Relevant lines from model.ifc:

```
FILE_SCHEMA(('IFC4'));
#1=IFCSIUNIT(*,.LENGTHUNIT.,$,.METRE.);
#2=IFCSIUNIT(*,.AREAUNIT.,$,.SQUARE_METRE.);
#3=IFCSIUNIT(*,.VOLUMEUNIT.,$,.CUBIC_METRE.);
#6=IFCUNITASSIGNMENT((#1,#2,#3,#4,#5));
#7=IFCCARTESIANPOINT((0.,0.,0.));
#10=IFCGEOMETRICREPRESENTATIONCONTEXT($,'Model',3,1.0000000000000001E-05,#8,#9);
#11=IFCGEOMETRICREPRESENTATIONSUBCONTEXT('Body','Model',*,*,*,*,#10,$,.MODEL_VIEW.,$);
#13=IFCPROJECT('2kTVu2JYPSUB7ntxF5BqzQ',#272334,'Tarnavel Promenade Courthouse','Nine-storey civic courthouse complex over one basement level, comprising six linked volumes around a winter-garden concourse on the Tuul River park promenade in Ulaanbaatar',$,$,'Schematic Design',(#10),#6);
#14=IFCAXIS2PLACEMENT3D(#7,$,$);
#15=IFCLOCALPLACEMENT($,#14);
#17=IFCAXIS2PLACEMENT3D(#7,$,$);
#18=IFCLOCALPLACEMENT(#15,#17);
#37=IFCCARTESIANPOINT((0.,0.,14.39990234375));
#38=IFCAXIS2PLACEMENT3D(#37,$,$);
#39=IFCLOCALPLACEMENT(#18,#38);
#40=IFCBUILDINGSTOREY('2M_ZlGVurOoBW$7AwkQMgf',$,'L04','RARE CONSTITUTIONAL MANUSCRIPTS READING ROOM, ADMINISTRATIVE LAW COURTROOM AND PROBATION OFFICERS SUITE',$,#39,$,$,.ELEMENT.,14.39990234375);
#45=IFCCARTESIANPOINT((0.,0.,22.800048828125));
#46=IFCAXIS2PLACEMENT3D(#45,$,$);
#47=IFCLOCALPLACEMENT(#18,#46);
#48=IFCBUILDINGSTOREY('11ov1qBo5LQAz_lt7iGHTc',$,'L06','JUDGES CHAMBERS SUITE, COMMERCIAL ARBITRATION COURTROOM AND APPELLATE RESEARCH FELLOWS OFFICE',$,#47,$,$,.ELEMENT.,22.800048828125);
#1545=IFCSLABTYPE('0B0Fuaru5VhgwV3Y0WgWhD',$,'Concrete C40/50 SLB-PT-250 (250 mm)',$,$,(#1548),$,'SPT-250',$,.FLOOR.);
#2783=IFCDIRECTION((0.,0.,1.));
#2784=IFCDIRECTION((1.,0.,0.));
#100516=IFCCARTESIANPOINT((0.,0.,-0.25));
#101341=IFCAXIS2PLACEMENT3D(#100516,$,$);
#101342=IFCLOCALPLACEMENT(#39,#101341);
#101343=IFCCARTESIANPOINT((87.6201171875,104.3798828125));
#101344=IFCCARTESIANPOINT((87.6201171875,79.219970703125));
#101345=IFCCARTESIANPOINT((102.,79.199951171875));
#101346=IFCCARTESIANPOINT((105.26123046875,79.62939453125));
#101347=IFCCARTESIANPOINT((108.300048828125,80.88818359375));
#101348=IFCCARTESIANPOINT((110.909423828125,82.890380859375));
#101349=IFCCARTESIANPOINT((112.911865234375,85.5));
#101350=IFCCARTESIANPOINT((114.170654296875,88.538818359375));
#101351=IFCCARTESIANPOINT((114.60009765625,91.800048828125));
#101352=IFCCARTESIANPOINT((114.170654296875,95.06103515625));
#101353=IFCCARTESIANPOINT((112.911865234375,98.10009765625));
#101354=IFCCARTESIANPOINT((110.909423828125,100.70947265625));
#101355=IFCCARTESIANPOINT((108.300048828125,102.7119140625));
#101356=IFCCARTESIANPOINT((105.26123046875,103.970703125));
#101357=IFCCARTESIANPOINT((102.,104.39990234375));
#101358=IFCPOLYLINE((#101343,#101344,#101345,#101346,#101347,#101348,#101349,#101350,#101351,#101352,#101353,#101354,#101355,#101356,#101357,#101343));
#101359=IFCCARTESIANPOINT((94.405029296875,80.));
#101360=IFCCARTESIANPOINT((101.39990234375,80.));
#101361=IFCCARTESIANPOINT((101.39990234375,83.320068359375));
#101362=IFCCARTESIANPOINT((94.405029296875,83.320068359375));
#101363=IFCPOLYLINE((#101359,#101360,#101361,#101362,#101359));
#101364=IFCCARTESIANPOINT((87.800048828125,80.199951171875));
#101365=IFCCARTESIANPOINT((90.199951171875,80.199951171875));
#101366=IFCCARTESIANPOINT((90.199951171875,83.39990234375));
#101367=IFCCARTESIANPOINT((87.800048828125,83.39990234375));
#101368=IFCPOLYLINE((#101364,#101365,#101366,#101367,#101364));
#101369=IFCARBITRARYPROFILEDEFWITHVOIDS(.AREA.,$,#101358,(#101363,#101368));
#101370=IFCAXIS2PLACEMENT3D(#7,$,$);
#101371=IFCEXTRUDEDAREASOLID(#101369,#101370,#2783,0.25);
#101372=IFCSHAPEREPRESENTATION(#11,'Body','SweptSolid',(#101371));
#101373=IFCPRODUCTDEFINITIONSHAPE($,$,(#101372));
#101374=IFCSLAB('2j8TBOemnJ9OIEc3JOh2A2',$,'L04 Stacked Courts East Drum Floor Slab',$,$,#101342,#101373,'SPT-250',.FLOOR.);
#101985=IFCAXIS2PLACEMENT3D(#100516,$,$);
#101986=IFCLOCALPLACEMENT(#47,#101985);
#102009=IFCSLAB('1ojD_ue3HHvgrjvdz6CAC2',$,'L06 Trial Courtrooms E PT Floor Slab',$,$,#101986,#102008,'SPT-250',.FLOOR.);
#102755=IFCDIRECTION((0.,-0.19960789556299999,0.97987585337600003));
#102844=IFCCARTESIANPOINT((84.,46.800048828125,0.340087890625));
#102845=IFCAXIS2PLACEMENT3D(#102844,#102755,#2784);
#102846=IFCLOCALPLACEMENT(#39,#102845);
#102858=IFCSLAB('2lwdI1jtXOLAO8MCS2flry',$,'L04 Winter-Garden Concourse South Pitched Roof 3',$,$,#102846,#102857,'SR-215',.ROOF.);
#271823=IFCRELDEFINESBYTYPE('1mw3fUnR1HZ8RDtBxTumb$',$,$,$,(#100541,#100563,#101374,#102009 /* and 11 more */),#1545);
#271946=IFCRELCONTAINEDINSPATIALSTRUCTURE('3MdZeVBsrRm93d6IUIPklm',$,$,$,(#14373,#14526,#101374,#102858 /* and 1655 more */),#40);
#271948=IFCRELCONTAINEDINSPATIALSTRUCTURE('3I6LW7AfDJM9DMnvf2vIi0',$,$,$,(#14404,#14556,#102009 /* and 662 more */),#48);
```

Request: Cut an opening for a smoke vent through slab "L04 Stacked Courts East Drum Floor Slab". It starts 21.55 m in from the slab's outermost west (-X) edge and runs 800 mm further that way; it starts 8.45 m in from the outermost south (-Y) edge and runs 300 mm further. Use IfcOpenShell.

```python
import numpy as np
import ifcopenshell
import ifcopenshell.api.feature
import ifcopenshell.api.geometry
import ifcopenshell.api.root
import ifcopenshell.geom
import ifcopenshell.util.placement
import ifcopenshell.util.representation
import ifcopenshell.util.shape
import ifcopenshell.util.unit

model = ifcopenshell.open("model.ifc")
unit_scale = ifcopenshell.util.unit.calculate_unit_scale(model)
settings = ifcopenshell.geom.settings()


def volume(element):
    """Net volume in cubic metres, openings subtracted."""
    shape = ifcopenshell.geom.create_shape(settings, element)
    return ifcopenshell.util.shape.get_volume(shape.geometry)


slab = model.by_guid("2j8TBOemnJ9OIEc3JOh2A2")
before = volume(slab)

# Extent in the slab's own axes, in metres. The edges named are its -X and -Y sides.
slab_shape = ifcopenshell.geom.create_shape(settings, slab)
vertices = ifcopenshell.util.shape.get_vertices(slab_shape.geometry)
x_min, y_min, bottom = vertices.min(axis=0)
top = vertices[:, 2].max()

opening = ifcopenshell.api.root.create_entity(model, ifc_class="IfcOpeningElement", name="Smoke vent opening", predefined_type="OPENING")
context = ifcopenshell.util.representation.get_context(model, "Model", "Body", "MODEL_VIEW")
width, depth = 0.8, 0.3
outline = [(0.0, 0.0), (width, 0.0), (width, depth), (0.0, depth), (0.0, 0.0)]
# Overshoot both faces by 50 mm so the cut is clean.
shape = ifcopenshell.api.geometry.add_slab_representation(
    model, context=context, depth=top - bottom + 0.1, polyline=outline
)
ifcopenshell.api.geometry.assign_representation(model, product=opening, representation=shape)

matrix = ifcopenshell.util.placement.get_local_placement(slab.ObjectPlacement)
matrix[:, 3] = matrix @ np.append(np.array([x_min + 21.55, y_min + 8.45, bottom - 0.05]) / unit_scale, 1.0)
ifcopenshell.api.geometry.edit_object_placement(model, product=opening, matrix=matrix, is_si=False)
ifcopenshell.api.feature.add_feature(model, feature=opening, element=slab)

after = volume(slab)

print(f"slab volume {before:.3f} -> {after:.3f} m3")

model.write("model-out.ifc")
```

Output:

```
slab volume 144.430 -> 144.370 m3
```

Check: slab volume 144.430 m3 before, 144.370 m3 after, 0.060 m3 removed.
